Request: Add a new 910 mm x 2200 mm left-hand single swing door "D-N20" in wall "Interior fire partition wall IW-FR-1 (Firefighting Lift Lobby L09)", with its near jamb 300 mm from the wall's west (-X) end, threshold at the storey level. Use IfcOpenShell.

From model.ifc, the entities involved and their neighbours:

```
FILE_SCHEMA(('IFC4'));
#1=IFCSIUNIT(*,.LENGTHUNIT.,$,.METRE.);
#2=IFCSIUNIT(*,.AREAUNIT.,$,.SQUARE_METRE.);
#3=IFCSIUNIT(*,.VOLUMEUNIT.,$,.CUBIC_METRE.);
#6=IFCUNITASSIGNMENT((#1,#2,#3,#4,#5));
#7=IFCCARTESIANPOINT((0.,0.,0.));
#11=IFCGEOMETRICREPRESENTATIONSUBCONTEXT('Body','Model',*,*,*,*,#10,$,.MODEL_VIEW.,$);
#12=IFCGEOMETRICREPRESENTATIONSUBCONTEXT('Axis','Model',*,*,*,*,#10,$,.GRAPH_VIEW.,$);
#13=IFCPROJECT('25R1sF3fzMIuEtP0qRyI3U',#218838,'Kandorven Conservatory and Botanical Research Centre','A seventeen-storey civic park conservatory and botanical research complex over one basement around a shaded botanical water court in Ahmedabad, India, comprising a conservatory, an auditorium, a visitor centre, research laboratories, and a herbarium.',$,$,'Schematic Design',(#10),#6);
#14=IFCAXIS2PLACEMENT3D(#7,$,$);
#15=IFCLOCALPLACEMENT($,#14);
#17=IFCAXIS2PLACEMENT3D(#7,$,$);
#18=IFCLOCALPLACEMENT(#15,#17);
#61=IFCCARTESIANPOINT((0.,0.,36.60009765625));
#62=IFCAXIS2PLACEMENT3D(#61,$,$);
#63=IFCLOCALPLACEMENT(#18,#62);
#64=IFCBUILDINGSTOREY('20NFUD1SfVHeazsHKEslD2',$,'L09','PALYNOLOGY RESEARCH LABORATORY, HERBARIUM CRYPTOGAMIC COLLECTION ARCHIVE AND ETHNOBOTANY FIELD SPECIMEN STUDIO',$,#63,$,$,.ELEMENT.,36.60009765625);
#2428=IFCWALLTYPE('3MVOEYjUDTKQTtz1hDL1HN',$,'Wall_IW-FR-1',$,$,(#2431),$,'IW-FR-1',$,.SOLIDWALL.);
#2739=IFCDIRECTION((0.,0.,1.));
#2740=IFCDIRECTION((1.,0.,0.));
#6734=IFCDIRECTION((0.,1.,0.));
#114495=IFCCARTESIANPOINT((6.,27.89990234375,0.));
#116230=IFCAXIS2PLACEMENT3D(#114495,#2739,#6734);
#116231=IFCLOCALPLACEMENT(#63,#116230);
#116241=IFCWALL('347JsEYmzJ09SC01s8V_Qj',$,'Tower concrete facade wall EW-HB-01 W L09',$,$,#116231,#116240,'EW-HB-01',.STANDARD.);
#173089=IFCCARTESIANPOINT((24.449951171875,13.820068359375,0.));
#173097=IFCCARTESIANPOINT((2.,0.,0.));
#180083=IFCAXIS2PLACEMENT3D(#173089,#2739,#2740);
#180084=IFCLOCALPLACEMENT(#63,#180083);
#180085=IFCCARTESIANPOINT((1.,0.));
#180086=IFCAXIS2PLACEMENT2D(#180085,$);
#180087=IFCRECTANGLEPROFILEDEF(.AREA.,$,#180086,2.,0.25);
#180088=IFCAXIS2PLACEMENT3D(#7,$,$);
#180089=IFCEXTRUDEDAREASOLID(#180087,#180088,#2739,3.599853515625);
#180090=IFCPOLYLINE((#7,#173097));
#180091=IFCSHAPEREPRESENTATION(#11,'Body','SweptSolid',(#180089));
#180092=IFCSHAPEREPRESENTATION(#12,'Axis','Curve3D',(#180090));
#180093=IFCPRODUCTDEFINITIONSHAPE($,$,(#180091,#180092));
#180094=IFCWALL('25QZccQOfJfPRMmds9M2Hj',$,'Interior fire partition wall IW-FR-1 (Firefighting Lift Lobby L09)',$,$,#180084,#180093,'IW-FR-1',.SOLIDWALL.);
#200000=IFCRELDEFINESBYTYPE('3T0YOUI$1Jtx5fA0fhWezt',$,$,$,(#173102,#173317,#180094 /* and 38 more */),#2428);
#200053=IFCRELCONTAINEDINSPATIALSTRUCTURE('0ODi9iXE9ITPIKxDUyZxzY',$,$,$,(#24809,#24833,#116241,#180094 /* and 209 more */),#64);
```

```python
import numpy as np
import ifcopenshell
import ifcopenshell.api.feature
import ifcopenshell.api.geometry
import ifcopenshell.api.root
import ifcopenshell.api.spatial
import ifcopenshell.geom
import ifcopenshell.util.element
import ifcopenshell.util.placement
import ifcopenshell.util.representation
import ifcopenshell.util.shape
import ifcopenshell.util.unit

model = ifcopenshell.open("model.ifc")
unit_scale = ifcopenshell.util.unit.calculate_unit_scale(model)
settings = ifcopenshell.geom.settings()


def volume(element):
    """Net volume in cubic metres, openings subtracted."""
    shape = ifcopenshell.geom.create_shape(settings, element)
    return ifcopenshell.util.shape.get_volume(shape.geometry)


wall = model.by_guid("25QZccQOfJfPRMmds9M2Hj")
storey = ifcopenshell.util.element.get_container(wall, ifc_class="IfcBuildingStorey")
context = ifcopenshell.util.representation.get_context(model, "Model", "Body", "MODEL_VIEW")
before = volume(wall)

width, height, from_end, sill = 0.91, 2.2, 0.3, 0.0  # metres

# The wall runs along its own X axis, and the end named is its -X end.
wall_shape = ifcopenshell.geom.create_shape(settings, wall)
x, y, z = ifcopenshell.util.shape.get_vertices(wall_shape.geometry).T
start = x.min() + from_end
face, thickness = float(y.min()), float(y.max() - y.min())
wall_matrix = ifcopenshell.util.placement.get_local_placement(wall.ObjectPlacement)
level = ifcopenshell.util.placement.get_local_placement(storey.ObjectPlacement)[2, 3]


def in_wall(x, y):
    """Placement at x, y metres in the wall's axes, at sill height."""
    matrix = wall_matrix.copy()
    matrix[:, 3] = wall_matrix @ np.array([x / unit_scale, y / unit_scale, 0.0, 1.0])
    matrix[2, 3] = level + sill / unit_scale
    return matrix


# Opening: a box that overshoots both wall faces by 50 mm.
opening = ifcopenshell.api.root.create_entity(model, ifc_class="IfcOpeningElement", predefined_type="OPENING")
box = ifcopenshell.api.geometry.add_wall_representation(
    model, context=context, length=width, height=height, thickness=thickness + 0.1
)
ifcopenshell.api.geometry.assign_representation(model, product=opening, representation=box)
ifcopenshell.api.geometry.edit_object_placement(model, product=opening, matrix=in_wall(start, face - 0.05), is_si=False)
ifcopenshell.api.feature.add_feature(model, feature=opening, element=wall)

door = ifcopenshell.api.root.create_entity(model, ifc_class="IfcDoor", name="D-N20", predefined_type="DOOR")
door.OverallWidth, door.OverallHeight = width / unit_scale, height / unit_scale
door.OperationType = "SINGLE_SWING_LEFT"
body = ifcopenshell.api.geometry.add_door_representation(
    model,
    context=context,
    overall_width=door.OverallWidth,
    overall_height=door.OverallHeight,
    operation_type="SINGLE_SWING_LEFT",
    lining_properties={"LiningDepth": thickness / unit_scale, "ThresholdDepth": thickness / unit_scale},
)
ifcopenshell.api.geometry.assign_representation(model, product=door, representation=body)
ifcopenshell.api.spatial.assign_container(model, products=[door], relating_structure=storey)
ifcopenshell.api.feature.add_filling(model, opening=opening, element=door)

# The lining spans the wall, so the door starts at the wall face.
ifcopenshell.api.geometry.edit_object_placement(model, product=door, matrix=in_wall(start, face), is_si=False)

after = volume(wall)

print(f"wall volume {before:.3f} -> {after:.3f} m3")

model.write("model_updated.ifc")
```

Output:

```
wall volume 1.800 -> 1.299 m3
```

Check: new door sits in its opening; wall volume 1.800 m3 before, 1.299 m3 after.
